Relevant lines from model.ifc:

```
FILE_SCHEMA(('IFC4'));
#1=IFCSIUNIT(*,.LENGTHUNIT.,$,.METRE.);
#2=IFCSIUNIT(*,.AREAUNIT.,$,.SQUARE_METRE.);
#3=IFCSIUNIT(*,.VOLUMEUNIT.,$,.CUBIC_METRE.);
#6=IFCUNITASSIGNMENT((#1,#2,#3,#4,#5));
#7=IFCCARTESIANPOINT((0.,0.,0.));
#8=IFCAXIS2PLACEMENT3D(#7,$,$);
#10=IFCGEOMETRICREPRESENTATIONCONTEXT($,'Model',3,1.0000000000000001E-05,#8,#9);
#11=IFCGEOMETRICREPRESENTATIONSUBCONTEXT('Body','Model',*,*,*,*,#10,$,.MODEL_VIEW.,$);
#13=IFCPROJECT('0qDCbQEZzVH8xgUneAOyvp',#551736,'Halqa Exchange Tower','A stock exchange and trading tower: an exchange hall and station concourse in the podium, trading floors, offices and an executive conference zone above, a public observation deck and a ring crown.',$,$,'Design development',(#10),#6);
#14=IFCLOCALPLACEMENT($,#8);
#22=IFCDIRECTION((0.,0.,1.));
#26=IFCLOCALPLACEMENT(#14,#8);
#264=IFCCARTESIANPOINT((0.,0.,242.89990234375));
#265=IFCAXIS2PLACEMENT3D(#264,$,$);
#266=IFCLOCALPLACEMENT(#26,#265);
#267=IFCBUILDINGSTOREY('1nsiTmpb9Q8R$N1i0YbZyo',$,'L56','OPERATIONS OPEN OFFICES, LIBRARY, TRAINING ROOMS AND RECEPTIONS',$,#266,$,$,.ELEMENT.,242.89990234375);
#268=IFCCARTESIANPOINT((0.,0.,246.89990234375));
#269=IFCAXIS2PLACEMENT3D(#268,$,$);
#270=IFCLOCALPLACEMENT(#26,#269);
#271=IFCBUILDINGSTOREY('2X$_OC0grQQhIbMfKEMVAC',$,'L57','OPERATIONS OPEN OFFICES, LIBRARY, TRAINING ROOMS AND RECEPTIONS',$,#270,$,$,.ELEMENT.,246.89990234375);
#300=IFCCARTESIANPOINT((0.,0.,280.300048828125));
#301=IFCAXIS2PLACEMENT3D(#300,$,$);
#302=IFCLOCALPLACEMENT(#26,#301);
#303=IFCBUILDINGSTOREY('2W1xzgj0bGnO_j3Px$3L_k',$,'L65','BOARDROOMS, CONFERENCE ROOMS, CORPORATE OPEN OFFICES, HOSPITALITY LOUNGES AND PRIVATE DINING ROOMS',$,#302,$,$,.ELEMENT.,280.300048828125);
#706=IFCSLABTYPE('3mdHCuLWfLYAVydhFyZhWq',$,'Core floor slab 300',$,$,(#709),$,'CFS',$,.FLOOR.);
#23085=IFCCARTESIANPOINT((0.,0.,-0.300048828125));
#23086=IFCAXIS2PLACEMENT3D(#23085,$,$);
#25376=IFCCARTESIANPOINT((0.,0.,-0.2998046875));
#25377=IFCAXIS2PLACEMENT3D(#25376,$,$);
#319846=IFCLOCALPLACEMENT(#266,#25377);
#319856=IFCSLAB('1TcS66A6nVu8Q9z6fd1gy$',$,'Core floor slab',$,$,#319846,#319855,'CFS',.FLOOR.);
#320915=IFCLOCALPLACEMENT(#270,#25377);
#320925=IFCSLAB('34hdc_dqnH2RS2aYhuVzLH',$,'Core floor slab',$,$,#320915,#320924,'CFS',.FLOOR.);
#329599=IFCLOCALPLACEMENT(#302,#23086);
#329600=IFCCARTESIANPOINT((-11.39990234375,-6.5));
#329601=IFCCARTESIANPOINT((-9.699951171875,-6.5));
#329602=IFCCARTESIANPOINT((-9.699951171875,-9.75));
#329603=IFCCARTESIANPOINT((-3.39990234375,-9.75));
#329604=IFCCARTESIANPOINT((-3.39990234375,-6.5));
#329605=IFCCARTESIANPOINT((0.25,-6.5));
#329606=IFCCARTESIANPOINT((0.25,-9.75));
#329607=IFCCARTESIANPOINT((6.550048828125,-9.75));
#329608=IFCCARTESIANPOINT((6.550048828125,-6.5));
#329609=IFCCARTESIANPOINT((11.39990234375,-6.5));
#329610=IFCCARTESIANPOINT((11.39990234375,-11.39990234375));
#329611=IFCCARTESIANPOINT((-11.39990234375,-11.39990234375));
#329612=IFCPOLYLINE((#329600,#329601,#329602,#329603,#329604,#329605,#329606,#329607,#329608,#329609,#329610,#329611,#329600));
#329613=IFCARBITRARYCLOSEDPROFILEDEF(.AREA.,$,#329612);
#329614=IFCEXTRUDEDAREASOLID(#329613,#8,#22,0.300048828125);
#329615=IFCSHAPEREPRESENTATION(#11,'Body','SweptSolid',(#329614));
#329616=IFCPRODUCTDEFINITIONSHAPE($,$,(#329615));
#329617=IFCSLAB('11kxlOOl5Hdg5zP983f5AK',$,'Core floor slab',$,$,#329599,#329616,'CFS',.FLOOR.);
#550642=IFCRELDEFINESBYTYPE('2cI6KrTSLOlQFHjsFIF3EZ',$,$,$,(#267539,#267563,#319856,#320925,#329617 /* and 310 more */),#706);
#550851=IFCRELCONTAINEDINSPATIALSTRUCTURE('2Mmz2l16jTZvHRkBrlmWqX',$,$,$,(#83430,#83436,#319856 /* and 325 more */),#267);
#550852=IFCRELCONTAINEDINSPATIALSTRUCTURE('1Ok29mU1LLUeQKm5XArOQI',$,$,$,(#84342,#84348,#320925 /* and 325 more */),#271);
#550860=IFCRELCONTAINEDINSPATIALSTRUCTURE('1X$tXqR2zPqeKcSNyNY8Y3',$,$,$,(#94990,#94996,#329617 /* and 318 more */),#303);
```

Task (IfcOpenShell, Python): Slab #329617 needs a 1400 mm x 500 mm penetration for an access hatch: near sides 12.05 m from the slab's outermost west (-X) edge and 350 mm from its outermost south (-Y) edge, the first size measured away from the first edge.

```python
import numpy as np
import ifcopenshell
import ifcopenshell.api.feature
import ifcopenshell.api.geometry
import ifcopenshell.api.root
import ifcopenshell.geom
import ifcopenshell.util.placement
import ifcopenshell.util.representation
import ifcopenshell.util.shape
import ifcopenshell.util.unit

model = ifcopenshell.open("model.ifc")
unit_scale = ifcopenshell.util.unit.calculate_unit_scale(model)
settings = ifcopenshell.geom.settings()


def volume(element):
    """Net volume in cubic metres, openings subtracted."""
    shape = ifcopenshell.geom.create_shape(settings, element)
    return ifcopenshell.util.shape.get_volume(shape.geometry)


slab = model.by_guid("11kxlOOl5Hdg5zP983f5AK")
before = volume(slab)

# Extent in the slab's own axes, in metres. The edges named are its -X and -Y sides.
slab_shape = ifcopenshell.geom.create_shape(settings, slab)
vertices = ifcopenshell.util.shape.get_vertices(slab_shape.geometry)
x_min, y_min, bottom = vertices.min(axis=0)
top = vertices[:, 2].max()

opening = ifcopenshell.api.root.create_entity(model, ifc_class="IfcOpeningElement", name="Access hatch opening", predefined_type="OPENING")
context = ifcopenshell.util.representation.get_context(model, "Model", "Body", "MODEL_VIEW")
width, depth = 1.4, 0.5
outline = [(0.0, 0.0), (width, 0.0), (width, depth), (0.0, depth), (0.0, 0.0)]
# Overshoot both faces by 50 mm so the cut is clean.
shape = ifcopenshell.api.geometry.add_slab_representation(
    model, context=context, depth=top - bottom + 0.1, polyline=outline
)
ifcopenshell.api.geometry.assign_representation(model, product=opening, representation=shape)

matrix = ifcopenshell.util.placement.get_local_placement(slab.ObjectPlacement)
matrix[:, 3] = matrix @ np.append(np.array([x_min + 12.05, y_min + 0.35, bottom - 0.05]) / unit_scale, 1.0)
ifcopenshell.api.geometry.edit_object_placement(model, product=opening, matrix=matrix, is_si=False)
ifcopenshell.api.feature.add_feature(model, feature=opening, element=slab)

after = volume(slab)

print(f"slab volume {before:.3f} -> {after:.3f} m3")

model.write("model_updated.ifc")
```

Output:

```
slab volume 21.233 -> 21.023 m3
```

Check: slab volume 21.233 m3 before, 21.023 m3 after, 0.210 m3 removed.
